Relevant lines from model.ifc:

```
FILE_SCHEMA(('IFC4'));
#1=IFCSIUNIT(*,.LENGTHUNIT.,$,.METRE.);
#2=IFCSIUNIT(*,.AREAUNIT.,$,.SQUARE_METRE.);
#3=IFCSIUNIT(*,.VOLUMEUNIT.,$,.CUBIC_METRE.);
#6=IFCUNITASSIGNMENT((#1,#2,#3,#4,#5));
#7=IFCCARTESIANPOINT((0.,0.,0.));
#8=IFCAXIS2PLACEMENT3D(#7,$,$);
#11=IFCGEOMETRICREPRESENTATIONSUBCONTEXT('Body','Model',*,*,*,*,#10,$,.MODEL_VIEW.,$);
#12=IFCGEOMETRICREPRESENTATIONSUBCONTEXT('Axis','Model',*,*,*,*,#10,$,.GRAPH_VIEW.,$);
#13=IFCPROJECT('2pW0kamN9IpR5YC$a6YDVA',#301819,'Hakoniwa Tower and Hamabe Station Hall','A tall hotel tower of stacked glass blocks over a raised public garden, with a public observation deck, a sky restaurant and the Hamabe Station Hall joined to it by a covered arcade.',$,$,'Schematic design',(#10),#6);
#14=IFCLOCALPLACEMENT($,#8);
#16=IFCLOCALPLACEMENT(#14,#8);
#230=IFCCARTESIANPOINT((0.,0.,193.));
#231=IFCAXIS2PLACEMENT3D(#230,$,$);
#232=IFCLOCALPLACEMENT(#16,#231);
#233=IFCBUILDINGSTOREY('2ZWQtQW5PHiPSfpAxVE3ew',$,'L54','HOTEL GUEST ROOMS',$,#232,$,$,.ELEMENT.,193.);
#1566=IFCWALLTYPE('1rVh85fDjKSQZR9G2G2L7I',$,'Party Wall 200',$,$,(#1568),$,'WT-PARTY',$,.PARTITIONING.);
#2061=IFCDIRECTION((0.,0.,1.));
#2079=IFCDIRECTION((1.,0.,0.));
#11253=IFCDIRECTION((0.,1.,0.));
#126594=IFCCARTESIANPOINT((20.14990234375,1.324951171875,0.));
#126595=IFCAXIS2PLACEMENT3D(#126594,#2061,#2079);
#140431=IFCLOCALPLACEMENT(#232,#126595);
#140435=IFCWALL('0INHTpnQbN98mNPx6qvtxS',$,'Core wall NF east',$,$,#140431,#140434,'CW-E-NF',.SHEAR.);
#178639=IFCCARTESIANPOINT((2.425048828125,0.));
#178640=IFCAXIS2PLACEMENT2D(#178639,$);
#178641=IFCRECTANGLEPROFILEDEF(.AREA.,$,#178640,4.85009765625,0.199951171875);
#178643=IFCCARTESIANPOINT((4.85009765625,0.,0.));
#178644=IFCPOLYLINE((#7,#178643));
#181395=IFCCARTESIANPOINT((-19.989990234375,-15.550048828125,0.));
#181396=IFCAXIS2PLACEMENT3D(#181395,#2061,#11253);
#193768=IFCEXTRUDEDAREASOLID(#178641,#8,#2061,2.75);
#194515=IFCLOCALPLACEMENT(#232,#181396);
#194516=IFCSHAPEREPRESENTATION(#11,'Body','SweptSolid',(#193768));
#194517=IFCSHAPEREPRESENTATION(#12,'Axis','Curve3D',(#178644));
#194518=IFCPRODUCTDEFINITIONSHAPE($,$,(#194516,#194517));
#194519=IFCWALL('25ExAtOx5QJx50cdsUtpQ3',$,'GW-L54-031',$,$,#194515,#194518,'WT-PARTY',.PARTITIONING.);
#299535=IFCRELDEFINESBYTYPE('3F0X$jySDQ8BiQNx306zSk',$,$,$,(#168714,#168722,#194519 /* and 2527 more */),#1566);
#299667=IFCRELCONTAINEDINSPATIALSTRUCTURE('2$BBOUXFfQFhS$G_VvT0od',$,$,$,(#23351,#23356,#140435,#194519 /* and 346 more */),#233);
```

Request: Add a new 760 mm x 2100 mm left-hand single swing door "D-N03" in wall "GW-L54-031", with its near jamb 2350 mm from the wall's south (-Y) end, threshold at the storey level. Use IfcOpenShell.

```python
import numpy as np
import ifcopenshell
import ifcopenshell.api.feature
import ifcopenshell.api.geometry
import ifcopenshell.api.root
import ifcopenshell.api.spatial
import ifcopenshell.geom
import ifcopenshell.util.element
import ifcopenshell.util.placement
import ifcopenshell.util.representation
import ifcopenshell.util.shape
import ifcopenshell.util.unit

model = ifcopenshell.open("model.ifc")
unit_scale = ifcopenshell.util.unit.calculate_unit_scale(model)
settings = ifcopenshell.geom.settings()


def volume(element):
    """Net volume in cubic metres, openings subtracted."""
    shape = ifcopenshell.geom.create_shape(settings, element)
    return ifcopenshell.util.shape.get_volume(shape.geometry)


wall = model.by_guid("25ExAtOx5QJx50cdsUtpQ3")
storey = ifcopenshell.util.element.get_container(wall, ifc_class="IfcBuildingStorey")
context = ifcopenshell.util.representation.get_context(model, "Model", "Body", "MODEL_VIEW")
before = volume(wall)

width, height, from_end, sill = 0.76, 2.1, 2.35, 0.0  # metres

# The wall runs along its own X axis, and the end named is its -X end.
wall_shape = ifcopenshell.geom.create_shape(settings, wall)
x, y, z = ifcopenshell.util.shape.get_vertices(wall_shape.geometry).T
start = x.min() + from_end
face, thickness = float(y.min()), float(y.max() - y.min())
wall_matrix = ifcopenshell.util.placement.get_local_placement(wall.ObjectPlacement)
level = ifcopenshell.util.placement.get_local_placement(storey.ObjectPlacement)[2, 3]


def in_wall(x, y):
    """Placement at x, y metres in the wall's axes, at sill height."""
    matrix = wall_matrix.copy()
    matrix[:, 3] = wall_matrix @ np.array([x / unit_scale, y / unit_scale, 0.0, 1.0])
    matrix[2, 3] = level + sill / unit_scale
    return matrix


# Opening: a box that overshoots both wall faces by 50 mm.
opening = ifcopenshell.api.root.create_entity(model, ifc_class="IfcOpeningElement", predefined_type="OPENING")
box = ifcopenshell.api.geometry.add_wall_representation(
    model, context=context, length=width, height=height, thickness=thickness + 0.1
)
ifcopenshell.api.geometry.assign_representation(model, product=opening, representation=box)
ifcopenshell.api.geometry.edit_object_placement(model, product=opening, matrix=in_wall(start, face - 0.05), is_si=False)
ifcopenshell.api.feature.add_feature(model, feature=opening, element=wall)

door = ifcopenshell.api.root.create_entity(model, ifc_class="IfcDoor", name="D-N03", predefined_type="DOOR")
door.OverallWidth, door.OverallHeight = width / unit_scale, height / unit_scale
door.OperationType = "SINGLE_SWING_LEFT"
body = ifcopenshell.api.geometry.add_door_representation(
    model,
    context=context,
    overall_width=door.OverallWidth,
    overall_height=door.OverallHeight,
    operation_type="SINGLE_SWING_LEFT",
    lining_properties={"LiningDepth": thickness / unit_scale, "ThresholdDepth": thickness / unit_scale},
)
ifcopenshell.api.geometry.assign_representation(model, product=door, representation=body)
ifcopenshell.api.spatial.assign_container(model, products=[door], relating_structure=storey)
ifcopenshell.api.feature.add_filling(model, opening=opening, element=door)

# The lining spans the wall, so the door starts at the wall face.
ifcopenshell.api.geometry.edit_object_placement(model, product=door, matrix=in_wall(start, face), is_si=False)

after = volume(wall)

print(f"wall volume {before:.3f} -> {after:.3f} m3")

model.write("model_v2.ifc")
```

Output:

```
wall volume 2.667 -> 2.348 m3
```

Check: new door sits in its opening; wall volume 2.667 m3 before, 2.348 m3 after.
